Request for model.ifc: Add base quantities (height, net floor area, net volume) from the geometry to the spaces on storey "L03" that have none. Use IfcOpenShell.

First a look at what the model holds.

```python
import ifcopenshell
import ifcopenshell.util.element
import ifcopenshell.util.unit

model = ifcopenshell.open("model.ifc")
print(model.schema)
for unit_type in ("LENGTHUNIT", "AREAUNIT", "VOLUMEUNIT"):
    print(unit_type, ifcopenshell.util.unit.calculate_unit_scale(model, unit_type))
storey = next(s for s in model.by_type("IfcBuildingStorey") if s.Name == "L03")
spaces = [e for e in ifcopenshell.util.element.get_decomposition(storey) if e.is_a("IfcSpace")]
for e in sorted(spaces, key=lambda e: e.id()):
    print(e.id(), e.is_a(), e.Name, list(ifcopenshell.util.element.get_psets(e, qtos_only=True)), sep=" | ")
```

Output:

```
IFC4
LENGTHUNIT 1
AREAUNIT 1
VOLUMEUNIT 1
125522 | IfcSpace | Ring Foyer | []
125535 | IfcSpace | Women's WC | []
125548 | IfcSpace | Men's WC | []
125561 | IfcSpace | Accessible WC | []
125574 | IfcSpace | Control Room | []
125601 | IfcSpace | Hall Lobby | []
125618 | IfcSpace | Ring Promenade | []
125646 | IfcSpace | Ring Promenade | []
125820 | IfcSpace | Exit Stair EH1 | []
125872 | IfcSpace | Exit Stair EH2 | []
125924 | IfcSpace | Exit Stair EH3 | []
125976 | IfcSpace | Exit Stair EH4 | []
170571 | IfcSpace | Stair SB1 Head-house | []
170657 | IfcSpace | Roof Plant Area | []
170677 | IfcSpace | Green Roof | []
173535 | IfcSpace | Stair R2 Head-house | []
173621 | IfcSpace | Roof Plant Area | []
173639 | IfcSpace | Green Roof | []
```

```python
import ifcopenshell
import ifcopenshell.api.pset
import ifcopenshell.geom
import ifcopenshell.util.element
import ifcopenshell.util.shape
import ifcopenshell.util.unit

model = ifcopenshell.open("model.ifc")
unit_scale = ifcopenshell.util.unit.calculate_unit_scale(model)
area_scale = ifcopenshell.util.unit.calculate_unit_scale(model, "AREAUNIT")
volume_scale = ifcopenshell.util.unit.calculate_unit_scale(model, "VOLUMEUNIT")
settings = ifcopenshell.geom.settings()

storey = next(s for s in model.by_type("IfcBuildingStorey") if s.Name == "L03")
spaces = [e for e in ifcopenshell.util.element.get_decomposition(storey) if e.is_a("IfcSpace")]

for e in sorted(spaces, key=lambda e: e.id()):
    if ifcopenshell.util.element.get_psets(e, qtos_only=True, should_inherit=False):
        continue
    # Geometry comes back in metres, in the element's own axes.
    shape = ifcopenshell.geom.create_shape(settings, e)
    values = {
        "Height": ifcopenshell.util.shape.get_z(shape.geometry) / unit_scale,
        "NetFloorArea": ifcopenshell.util.shape.get_footprint_area(shape.geometry) / area_scale,
        "NetVolume": ifcopenshell.util.shape.get_volume(shape.geometry) / volume_scale,
    }
    qto = ifcopenshell.api.pset.add_qto(model, product=e, name="Qto_SpaceBaseQuantities")
    ifcopenshell.api.pset.edit_qto(model, qto=qto, properties=values)
    print(e.id(), {k: round(v, 3) for k, v in values.items()})

model.write("model_edited.ifc")
```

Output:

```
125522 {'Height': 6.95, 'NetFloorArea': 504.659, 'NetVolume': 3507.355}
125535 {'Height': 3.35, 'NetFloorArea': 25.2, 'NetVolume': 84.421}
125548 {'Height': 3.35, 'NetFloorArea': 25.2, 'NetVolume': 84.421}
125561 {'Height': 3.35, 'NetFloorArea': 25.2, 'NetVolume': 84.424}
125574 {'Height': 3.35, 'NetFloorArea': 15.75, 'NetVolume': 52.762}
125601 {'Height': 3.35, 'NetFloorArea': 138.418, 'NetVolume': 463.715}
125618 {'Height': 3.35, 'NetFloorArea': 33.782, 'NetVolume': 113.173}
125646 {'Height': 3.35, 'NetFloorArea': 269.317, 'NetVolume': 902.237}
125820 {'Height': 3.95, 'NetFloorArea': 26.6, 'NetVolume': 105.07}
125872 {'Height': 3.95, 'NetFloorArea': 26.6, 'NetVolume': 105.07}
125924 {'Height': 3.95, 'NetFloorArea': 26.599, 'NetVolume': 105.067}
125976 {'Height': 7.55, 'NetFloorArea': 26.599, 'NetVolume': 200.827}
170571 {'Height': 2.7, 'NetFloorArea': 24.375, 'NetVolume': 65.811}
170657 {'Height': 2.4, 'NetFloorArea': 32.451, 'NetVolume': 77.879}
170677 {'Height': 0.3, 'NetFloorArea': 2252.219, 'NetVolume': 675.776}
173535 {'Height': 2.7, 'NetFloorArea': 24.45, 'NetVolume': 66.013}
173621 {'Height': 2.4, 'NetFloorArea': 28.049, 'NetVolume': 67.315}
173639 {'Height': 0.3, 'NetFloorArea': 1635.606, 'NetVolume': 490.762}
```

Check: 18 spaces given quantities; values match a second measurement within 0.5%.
